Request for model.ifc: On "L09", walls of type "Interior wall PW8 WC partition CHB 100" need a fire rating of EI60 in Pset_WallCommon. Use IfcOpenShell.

First a look at what the model holds.

```python
import ifcopenshell
import ifcopenshell.util.element

model = ifcopenshell.open("model.ifc")
print(model.schema)
storey = next(s for s in model.by_type("IfcBuildingStorey") if s.Name == "L09")
walls = [e for e in ifcopenshell.util.element.get_decomposition(storey) if e.is_a("IfcWall")]
seen = {}
for e in walls:
    element_type = ifcopenshell.util.element.get_type(e)
    key = (element_type.Name if element_type != e and element_type else None, ifcopenshell.util.element.get_pset(e, "Pset_WallCommon", "FireRating"))
    seen[key] = seen.get(key, 0) + 1
for (name, value), count in sorted(seen.items(), key=str):
    print(count, "x", name, "|", value)
```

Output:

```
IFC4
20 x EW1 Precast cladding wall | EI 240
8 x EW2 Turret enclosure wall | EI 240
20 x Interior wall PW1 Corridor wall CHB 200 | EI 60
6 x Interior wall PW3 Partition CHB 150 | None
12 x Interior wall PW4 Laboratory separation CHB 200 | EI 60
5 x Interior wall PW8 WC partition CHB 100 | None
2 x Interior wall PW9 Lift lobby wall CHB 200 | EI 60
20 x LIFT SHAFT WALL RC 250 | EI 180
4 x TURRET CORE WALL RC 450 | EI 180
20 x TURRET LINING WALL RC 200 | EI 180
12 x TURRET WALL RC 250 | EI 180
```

```python
import ifcopenshell
import ifcopenshell.api.pset
import ifcopenshell.util.element

model = ifcopenshell.open("model.ifc")

storey = next(s for s in model.by_type("IfcBuildingStorey") if s.Name == "L09")
walls = [e for e in ifcopenshell.util.element.get_decomposition(storey) if e.is_a("IfcWall")]

count = 0
for e in walls:
    element_type = ifcopenshell.util.element.get_type(e)
    if element_type in (None, e) or element_type.Name != "Interior wall PW8 WC partition CHB 100":
        continue
    # add_pset returns the element's existing set when there is one.
    pset = ifcopenshell.api.pset.add_pset(model, product=e, name="Pset_WallCommon")
    ifcopenshell.api.pset.edit_pset(model, pset=pset, properties={"FireRating": "EI60"})
    count += 1

print(count, "walls updated")

model.write("model-out.ifc")
```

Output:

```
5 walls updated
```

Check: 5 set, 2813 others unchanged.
